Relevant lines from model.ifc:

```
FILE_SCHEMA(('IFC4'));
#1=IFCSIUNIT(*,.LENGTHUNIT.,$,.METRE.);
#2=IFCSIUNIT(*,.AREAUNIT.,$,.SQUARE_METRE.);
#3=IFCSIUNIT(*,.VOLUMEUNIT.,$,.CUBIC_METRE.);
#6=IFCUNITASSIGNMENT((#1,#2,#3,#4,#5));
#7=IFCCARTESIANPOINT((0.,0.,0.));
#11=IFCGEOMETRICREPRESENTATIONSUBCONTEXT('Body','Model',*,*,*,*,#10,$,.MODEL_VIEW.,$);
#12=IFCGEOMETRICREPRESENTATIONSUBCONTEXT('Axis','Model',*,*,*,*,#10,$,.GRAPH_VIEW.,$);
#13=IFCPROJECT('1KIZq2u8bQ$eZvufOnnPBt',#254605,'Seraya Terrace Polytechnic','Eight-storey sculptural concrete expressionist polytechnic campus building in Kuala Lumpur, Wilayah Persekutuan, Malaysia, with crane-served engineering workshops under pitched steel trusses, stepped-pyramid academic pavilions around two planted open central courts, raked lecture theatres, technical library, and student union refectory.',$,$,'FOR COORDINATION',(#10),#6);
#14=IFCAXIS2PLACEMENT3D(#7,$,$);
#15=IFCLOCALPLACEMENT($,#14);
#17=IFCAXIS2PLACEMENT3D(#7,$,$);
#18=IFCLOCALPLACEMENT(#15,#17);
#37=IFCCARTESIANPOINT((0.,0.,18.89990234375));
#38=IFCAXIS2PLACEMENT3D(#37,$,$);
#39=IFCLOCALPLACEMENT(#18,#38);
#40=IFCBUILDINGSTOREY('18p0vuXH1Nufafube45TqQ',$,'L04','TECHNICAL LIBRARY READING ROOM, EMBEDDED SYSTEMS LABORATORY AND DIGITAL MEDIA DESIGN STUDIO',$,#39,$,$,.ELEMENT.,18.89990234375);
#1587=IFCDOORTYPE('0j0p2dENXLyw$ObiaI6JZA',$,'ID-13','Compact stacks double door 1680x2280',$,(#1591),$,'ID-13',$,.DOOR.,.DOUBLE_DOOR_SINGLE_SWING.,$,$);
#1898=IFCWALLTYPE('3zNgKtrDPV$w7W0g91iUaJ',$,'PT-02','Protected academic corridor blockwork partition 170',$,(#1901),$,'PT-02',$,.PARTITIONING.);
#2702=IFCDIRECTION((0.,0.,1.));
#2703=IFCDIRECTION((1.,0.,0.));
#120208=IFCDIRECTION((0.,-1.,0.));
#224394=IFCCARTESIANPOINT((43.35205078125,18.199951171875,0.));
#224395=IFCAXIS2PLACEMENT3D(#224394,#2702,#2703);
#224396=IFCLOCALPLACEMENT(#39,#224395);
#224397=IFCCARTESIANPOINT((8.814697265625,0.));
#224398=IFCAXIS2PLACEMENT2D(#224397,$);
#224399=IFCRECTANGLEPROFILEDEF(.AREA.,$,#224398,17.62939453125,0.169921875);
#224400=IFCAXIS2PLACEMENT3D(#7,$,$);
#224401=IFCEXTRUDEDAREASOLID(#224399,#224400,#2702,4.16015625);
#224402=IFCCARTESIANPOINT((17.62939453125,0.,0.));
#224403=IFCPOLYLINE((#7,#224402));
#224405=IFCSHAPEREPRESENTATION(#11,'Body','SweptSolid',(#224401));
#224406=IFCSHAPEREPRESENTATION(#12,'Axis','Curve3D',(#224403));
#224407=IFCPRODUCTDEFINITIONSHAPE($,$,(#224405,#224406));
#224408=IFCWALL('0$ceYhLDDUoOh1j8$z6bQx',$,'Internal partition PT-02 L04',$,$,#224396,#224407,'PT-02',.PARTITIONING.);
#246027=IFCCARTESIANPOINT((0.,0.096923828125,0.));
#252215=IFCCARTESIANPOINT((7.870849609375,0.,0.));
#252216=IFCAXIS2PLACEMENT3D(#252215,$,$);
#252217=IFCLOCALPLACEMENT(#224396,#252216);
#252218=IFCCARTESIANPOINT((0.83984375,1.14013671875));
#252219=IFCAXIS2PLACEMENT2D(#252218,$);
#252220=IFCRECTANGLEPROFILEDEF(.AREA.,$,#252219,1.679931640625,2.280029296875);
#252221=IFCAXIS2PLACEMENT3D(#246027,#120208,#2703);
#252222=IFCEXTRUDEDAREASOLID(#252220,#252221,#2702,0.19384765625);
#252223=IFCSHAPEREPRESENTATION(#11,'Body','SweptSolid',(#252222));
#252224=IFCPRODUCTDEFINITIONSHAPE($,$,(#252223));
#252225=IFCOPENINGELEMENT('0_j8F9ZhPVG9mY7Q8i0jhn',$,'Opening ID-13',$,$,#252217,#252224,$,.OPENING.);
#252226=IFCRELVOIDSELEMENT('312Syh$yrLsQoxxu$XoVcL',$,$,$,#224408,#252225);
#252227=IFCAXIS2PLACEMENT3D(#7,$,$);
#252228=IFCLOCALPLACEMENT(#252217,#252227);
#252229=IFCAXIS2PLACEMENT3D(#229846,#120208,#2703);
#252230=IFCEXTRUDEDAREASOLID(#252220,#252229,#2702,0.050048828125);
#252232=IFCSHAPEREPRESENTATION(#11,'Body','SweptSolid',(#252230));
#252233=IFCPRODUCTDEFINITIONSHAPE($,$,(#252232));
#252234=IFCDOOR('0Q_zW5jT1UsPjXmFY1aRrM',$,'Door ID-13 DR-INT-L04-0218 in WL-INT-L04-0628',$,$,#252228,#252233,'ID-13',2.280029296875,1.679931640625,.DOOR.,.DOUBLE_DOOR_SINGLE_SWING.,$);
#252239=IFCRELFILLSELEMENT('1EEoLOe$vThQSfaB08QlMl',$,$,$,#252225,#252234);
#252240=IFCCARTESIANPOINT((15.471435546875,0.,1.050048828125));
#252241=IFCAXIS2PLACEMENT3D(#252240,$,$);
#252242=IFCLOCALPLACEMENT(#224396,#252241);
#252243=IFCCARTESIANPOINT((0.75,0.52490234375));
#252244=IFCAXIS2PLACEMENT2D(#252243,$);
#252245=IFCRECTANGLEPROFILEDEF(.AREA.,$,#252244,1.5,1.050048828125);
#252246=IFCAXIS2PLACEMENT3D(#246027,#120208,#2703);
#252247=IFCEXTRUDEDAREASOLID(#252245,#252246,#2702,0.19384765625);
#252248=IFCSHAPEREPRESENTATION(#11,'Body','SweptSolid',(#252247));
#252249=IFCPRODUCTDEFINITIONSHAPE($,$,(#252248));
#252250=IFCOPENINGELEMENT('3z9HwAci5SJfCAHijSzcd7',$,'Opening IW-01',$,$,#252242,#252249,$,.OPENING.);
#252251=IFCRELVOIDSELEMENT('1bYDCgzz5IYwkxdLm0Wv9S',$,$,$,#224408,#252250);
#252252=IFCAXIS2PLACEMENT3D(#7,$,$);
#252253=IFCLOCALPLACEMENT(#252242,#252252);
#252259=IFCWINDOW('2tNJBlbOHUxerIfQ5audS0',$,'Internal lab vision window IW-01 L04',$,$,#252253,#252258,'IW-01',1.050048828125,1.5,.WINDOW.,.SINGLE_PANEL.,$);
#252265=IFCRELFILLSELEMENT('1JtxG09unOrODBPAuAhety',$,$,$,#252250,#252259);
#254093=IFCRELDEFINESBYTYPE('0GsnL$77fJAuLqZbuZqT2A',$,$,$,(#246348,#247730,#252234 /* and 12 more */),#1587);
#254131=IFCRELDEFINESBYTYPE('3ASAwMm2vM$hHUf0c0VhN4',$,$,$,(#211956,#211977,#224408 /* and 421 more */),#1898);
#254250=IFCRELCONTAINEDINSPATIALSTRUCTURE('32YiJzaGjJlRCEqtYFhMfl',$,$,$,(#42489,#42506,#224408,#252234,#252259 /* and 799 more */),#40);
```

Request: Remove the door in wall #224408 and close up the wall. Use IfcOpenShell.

```python
import ifcopenshell
import ifcopenshell.api.feature
import ifcopenshell.api.root
import ifcopenshell.geom
import ifcopenshell.util.shape

model = ifcopenshell.open("model.ifc")
settings = ifcopenshell.geom.settings()


def volume(element):
    """Net volume in cubic metres, openings subtracted."""
    shape = ifcopenshell.geom.create_shape(settings, element)
    return ifcopenshell.util.shape.get_volume(shape.geometry)


door = model.by_guid("0Q_zW5jT1UsPjXmFY1aRrM")
opening = door.FillsVoids[0].RelatingOpeningElement
wall = opening.VoidsElements[0].RelatingBuildingElement
before = volume(wall)

ifcopenshell.api.root.remove_product(model, product=door)
ifcopenshell.api.feature.remove_feature(model, feature=opening)

after = volume(wall)

print(f"wall volume {before:.3f} -> {after:.3f} m3")

model.write("model-out.ifc")
```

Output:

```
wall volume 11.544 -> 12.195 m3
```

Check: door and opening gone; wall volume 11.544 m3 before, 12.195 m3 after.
